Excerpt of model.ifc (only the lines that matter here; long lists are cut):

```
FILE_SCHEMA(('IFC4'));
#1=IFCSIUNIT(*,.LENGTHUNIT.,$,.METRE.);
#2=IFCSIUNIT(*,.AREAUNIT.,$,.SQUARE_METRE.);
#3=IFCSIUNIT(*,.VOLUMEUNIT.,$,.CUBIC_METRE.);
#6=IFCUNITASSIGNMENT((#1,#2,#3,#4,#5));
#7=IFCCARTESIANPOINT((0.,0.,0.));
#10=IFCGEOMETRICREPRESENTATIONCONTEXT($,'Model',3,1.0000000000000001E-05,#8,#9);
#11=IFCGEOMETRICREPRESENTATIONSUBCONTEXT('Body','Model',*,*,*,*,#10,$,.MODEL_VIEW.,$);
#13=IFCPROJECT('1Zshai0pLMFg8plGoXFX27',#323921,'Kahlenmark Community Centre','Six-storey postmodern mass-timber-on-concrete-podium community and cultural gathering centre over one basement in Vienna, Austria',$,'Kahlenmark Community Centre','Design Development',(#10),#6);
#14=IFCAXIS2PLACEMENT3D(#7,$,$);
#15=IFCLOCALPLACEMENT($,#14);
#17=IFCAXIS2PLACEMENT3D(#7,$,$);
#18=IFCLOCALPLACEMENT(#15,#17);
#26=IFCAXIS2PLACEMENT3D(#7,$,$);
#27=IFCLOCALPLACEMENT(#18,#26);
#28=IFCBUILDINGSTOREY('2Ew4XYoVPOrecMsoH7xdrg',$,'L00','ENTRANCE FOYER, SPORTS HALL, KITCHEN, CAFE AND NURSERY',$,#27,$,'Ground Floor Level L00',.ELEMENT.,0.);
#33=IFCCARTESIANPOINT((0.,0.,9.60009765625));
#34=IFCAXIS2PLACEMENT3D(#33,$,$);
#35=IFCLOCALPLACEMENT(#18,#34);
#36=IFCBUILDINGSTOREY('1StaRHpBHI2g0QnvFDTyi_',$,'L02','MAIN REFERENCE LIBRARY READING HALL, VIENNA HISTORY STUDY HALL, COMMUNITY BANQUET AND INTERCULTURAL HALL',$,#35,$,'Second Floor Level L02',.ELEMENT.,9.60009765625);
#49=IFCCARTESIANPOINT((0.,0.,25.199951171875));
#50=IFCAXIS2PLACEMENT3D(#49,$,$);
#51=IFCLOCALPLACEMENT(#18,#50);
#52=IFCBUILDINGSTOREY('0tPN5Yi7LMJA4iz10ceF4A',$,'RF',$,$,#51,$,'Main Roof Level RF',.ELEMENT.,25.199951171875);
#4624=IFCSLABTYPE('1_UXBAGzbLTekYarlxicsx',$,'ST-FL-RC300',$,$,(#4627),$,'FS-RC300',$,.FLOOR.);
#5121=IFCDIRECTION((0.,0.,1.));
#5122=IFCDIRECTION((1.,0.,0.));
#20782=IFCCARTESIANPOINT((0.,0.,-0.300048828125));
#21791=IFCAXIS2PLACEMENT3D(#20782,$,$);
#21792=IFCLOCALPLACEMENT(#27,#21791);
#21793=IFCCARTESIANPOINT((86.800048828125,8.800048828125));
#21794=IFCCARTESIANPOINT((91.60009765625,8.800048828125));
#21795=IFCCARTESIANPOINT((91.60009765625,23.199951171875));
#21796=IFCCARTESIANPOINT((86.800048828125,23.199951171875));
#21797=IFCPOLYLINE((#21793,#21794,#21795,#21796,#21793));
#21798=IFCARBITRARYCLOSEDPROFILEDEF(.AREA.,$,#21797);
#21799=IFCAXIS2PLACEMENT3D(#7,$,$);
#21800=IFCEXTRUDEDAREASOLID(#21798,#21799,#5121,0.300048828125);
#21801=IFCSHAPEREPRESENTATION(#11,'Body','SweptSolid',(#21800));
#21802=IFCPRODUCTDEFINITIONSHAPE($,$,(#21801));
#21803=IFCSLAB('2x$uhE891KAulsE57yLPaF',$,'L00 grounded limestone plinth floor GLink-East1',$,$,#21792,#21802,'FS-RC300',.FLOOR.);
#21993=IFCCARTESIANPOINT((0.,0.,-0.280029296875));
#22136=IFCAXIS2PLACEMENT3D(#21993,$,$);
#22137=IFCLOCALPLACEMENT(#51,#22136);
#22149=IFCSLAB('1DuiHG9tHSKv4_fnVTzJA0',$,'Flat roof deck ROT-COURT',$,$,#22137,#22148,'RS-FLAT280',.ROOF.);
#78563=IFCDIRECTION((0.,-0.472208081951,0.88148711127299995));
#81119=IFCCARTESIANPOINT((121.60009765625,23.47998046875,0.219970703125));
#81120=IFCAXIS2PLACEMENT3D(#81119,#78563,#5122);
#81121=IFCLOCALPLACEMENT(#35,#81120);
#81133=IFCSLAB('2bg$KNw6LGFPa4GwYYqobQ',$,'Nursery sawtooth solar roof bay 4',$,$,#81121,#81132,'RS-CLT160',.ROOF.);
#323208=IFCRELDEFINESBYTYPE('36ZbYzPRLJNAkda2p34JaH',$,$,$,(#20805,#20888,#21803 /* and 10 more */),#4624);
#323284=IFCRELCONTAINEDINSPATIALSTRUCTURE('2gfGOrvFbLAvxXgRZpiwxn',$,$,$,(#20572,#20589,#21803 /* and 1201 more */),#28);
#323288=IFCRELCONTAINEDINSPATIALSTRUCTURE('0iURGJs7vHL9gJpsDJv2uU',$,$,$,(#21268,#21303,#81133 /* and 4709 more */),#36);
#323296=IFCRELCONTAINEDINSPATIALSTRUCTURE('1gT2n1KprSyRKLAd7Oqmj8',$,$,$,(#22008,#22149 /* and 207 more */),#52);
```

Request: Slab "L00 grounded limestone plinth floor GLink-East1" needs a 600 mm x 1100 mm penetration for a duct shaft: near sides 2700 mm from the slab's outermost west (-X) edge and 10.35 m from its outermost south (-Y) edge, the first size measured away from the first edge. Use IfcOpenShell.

```python
import numpy as np
import ifcopenshell
import ifcopenshell.api.feature
import ifcopenshell.api.geometry
import ifcopenshell.api.root
import ifcopenshell.geom
import ifcopenshell.util.placement
import ifcopenshell.util.representation
import ifcopenshell.util.shape
import ifcopenshell.util.unit

model = ifcopenshell.open("model.ifc")
unit_scale = ifcopenshell.util.unit.calculate_unit_scale(model)
settings = ifcopenshell.geom.settings()


def volume(element):
    """Net volume in cubic metres, openings subtracted."""
    shape = ifcopenshell.geom.create_shape(settings, element)
    return ifcopenshell.util.shape.get_volume(shape.geometry)


slab = model.by_guid("2x$uhE891KAulsE57yLPaF")
before = volume(slab)

# Extent in the slab's own axes, in metres. The edges named are its -X and -Y sides.
slab_shape = ifcopenshell.geom.create_shape(settings, slab)
vertices = ifcopenshell.util.shape.get_vertices(slab_shape.geometry)
x_min, y_min, bottom = vertices.min(axis=0)
top = vertices[:, 2].max()

opening = ifcopenshell.api.root.create_entity(model, ifc_class="IfcOpeningElement", name="Duct shaft opening", predefined_type="OPENING")
context = ifcopenshell.util.representation.get_context(model, "Model", "Body", "MODEL_VIEW")
width, depth = 0.6, 1.1
outline = [(0.0, 0.0), (width, 0.0), (width, depth), (0.0, depth), (0.0, 0.0)]
# Overshoot both faces by 50 mm so the cut is clean.
shape = ifcopenshell.api.geometry.add_slab_representation(
    model, context=context, depth=top - bottom + 0.1, polyline=outline
)
ifcopenshell.api.geometry.assign_representation(model, product=opening, representation=shape)

matrix = ifcopenshell.util.placement.get_local_placement(slab.ObjectPlacement)
matrix[:, 3] = matrix @ np.append(np.array([x_min + 2.7, y_min + 10.35, bottom - 0.05]) / unit_scale, 1.0)
ifcopenshell.api.geometry.edit_object_placement(model, product=opening, matrix=matrix, is_si=False)
ifcopenshell.api.feature.add_feature(model, feature=opening, element=slab)

after = volume(slab)

print(f"slab volume {before:.3f} -> {after:.3f} m3")

model.write("model_v2.ifc")
```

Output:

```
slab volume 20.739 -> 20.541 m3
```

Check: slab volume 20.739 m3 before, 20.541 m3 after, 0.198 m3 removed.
